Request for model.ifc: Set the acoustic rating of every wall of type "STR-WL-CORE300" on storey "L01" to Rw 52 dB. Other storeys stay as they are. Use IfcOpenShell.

First a look at what the model holds.

```python
import ifcopenshell
import ifcopenshell.util.element

model = ifcopenshell.open("model.ifc")
print(model.schema)
storey = next(s for s in model.by_type("IfcBuildingStorey") if s.Name == "L01")
walls = [e for e in ifcopenshell.util.element.get_decomposition(storey) if e.is_a("IfcWall")]
seen = {}
for e in walls:
    element_type = ifcopenshell.util.element.get_type(e)
    key = (element_type.Name if element_type != e and element_type else None, ifcopenshell.util.element.get_pset(e, "Pset_WallCommon", "AcousticRating"))
    seen[key] = seen.get(key, 0) + 1
for (name, value), count in sorted(seen.items(), key=str):
    print(count, "x", name, "|", value)
```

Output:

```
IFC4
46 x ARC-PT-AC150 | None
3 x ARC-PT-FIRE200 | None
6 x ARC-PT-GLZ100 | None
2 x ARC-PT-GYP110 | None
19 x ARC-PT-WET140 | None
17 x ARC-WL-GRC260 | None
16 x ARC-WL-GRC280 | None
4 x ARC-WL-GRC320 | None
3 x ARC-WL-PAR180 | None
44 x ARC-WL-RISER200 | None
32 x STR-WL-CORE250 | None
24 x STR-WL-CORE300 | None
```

```python
import ifcopenshell
import ifcopenshell.api.pset
import ifcopenshell.util.element

model = ifcopenshell.open("model.ifc")

storey = next(s for s in model.by_type("IfcBuildingStorey") if s.Name == "L01")
walls = [e for e in ifcopenshell.util.element.get_decomposition(storey) if e.is_a("IfcWall")]

count = 0
for e in walls:
    element_type = ifcopenshell.util.element.get_type(e)
    if element_type in (None, e) or element_type.Name != "STR-WL-CORE300":
        continue
    # add_pset returns the element's existing set when there is one.
    pset = ifcopenshell.api.pset.add_pset(model, product=e, name="Pset_WallCommon")
    ifcopenshell.api.pset.edit_pset(model, pset=pset, properties={"AcousticRating": "Rw 52 dB"})
    count += 1

print(count, "walls updated")

model.write("model_updated.ifc")
```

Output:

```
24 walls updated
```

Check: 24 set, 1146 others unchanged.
